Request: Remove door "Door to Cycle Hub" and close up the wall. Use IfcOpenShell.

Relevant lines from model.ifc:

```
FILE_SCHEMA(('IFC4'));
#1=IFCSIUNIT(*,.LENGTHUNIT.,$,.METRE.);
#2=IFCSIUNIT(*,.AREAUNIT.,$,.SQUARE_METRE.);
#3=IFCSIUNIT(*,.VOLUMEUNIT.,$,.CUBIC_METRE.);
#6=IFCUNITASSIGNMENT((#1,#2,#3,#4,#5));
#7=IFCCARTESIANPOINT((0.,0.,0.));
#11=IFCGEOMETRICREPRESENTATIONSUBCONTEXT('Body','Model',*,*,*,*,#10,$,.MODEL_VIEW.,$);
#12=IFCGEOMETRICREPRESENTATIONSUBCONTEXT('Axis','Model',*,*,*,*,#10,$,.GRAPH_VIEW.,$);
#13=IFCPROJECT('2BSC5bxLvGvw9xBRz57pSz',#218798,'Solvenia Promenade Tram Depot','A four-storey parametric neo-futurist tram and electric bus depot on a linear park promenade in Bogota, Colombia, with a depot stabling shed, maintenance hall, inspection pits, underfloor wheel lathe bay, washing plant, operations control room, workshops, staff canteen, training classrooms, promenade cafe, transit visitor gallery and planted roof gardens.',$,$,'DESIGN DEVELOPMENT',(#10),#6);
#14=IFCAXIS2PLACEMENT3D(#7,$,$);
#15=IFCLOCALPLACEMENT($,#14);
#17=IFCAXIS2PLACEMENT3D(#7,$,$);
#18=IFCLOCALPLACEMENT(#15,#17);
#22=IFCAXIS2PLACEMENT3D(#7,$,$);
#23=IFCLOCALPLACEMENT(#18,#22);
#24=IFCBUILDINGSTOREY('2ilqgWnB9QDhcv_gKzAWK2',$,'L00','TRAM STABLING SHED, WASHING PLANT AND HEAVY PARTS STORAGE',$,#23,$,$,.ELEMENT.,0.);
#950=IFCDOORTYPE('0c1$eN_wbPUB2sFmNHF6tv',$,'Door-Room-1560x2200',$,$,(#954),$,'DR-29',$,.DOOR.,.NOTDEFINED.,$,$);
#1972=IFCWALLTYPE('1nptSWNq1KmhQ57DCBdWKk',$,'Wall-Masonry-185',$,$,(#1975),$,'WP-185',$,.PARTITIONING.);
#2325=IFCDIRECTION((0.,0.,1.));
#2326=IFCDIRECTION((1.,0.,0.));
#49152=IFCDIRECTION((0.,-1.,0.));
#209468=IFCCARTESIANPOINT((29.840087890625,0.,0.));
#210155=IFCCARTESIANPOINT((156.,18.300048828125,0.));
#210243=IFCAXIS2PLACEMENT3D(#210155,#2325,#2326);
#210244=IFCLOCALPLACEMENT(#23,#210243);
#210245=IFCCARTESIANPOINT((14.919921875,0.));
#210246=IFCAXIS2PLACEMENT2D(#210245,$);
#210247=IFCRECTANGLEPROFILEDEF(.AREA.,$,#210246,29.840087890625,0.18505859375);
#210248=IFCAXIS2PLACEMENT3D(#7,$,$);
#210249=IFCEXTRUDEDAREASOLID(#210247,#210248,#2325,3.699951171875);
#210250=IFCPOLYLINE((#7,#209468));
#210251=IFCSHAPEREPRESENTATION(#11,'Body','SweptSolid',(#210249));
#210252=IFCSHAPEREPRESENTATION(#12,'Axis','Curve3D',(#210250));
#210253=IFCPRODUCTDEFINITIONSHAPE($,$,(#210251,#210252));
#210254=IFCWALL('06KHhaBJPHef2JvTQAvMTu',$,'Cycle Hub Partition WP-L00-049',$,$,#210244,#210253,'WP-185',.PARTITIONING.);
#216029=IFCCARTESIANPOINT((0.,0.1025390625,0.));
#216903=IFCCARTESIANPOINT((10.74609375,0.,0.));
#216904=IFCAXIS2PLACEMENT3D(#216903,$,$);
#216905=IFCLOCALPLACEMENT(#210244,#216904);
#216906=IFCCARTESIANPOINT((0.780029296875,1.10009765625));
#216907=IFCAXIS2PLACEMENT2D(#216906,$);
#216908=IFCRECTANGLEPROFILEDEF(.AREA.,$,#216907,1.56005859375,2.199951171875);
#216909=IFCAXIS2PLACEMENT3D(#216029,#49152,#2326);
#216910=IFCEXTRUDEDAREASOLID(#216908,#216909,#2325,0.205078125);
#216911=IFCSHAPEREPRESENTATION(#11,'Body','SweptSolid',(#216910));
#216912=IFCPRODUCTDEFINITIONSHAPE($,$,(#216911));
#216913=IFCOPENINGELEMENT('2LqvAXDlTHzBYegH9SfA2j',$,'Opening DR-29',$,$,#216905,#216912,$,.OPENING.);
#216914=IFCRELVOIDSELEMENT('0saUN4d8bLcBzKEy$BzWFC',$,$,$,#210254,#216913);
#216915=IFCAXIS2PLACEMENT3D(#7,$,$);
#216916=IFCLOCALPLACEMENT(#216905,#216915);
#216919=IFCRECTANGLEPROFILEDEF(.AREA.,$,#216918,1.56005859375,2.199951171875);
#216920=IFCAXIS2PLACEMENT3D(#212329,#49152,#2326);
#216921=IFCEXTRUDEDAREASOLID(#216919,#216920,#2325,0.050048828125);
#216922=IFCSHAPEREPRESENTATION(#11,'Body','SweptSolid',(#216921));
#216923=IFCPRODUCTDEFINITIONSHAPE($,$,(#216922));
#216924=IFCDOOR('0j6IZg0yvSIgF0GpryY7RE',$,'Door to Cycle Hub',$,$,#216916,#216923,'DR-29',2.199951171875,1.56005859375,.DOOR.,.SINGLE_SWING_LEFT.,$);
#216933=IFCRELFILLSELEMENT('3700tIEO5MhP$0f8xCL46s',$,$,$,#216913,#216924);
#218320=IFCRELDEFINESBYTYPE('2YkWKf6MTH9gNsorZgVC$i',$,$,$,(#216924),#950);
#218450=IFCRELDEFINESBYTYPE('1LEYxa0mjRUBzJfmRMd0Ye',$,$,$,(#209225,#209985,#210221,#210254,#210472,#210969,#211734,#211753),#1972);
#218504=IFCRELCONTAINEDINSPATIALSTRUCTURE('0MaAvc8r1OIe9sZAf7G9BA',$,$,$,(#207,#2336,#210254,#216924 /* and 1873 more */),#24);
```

```python
import ifcopenshell
import ifcopenshell.api.feature
import ifcopenshell.api.root
import ifcopenshell.geom
import ifcopenshell.util.shape

model = ifcopenshell.open("model.ifc")
settings = ifcopenshell.geom.settings()


def volume(element):
    """Net volume in cubic metres, openings subtracted."""
    shape = ifcopenshell.geom.create_shape(settings, element)
    return ifcopenshell.util.shape.get_volume(shape.geometry)


door = model.by_guid("0j6IZg0yvSIgF0GpryY7RE")
opening = door.FillsVoids[0].RelatingOpeningElement
wall = opening.VoidsElements[0].RelatingBuildingElement
before = volume(wall)

ifcopenshell.api.root.remove_product(model, product=door)
ifcopenshell.api.feature.remove_feature(model, feature=opening)

after = volume(wall)

print(f"wall volume {before:.3f} -> {after:.3f} m3")

model.write("model_edited.ifc")
```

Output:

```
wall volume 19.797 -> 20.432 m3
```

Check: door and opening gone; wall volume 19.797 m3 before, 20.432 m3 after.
